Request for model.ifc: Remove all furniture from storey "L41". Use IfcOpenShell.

First a look at what the model holds.

```python
import ifcopenshell
import ifcopenshell.util.element

model = ifcopenshell.open("model.ifc")
print(model.schema)
storey = next(s for s in model.by_type("IfcBuildingStorey") if s.Name == "L41")
furniture = [e for e in ifcopenshell.util.element.get_decomposition(storey) if e.is_a("IfcFurnishingElement")]
seen = {}
for e in furniture:
    element_type = ifcopenshell.util.element.get_type(e)
    name = element_type.Name if element_type not in (None, e) else None
    seen[name] = seen.get(name, 0) + 1
for name, count in sorted(seen.items(), key=str):
    print(count, "x", name)
```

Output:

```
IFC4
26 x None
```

```python
import ifcopenshell
import ifcopenshell.api.root
import ifcopenshell.util.element

model = ifcopenshell.open("model.ifc")

storey = next(s for s in model.by_type("IfcBuildingStorey") if s.Name == "L41")
furniture = [e for e in ifcopenshell.util.element.get_decomposition(storey) if e.is_a("IfcFurnishingElement")]

for e in furniture:
    ifcopenshell.api.root.remove_product(model, product=e)
print(len(furniture), "removed")

model.write("model_rev.ifc")
```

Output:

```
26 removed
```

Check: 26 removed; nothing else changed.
